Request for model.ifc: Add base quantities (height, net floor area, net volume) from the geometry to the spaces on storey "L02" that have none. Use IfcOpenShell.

First a look at what the model holds.

```python
import ifcopenshell
import ifcopenshell.util.element
import ifcopenshell.util.unit

model = ifcopenshell.open("model.ifc")
print(model.schema)
for unit_type in ("LENGTHUNIT", "AREAUNIT", "VOLUMEUNIT"):
    print(unit_type, ifcopenshell.util.unit.calculate_unit_scale(model, unit_type))
storey = next(s for s in model.by_type("IfcBuildingStorey") if s.Name == "L02")
spaces = [e for e in ifcopenshell.util.element.get_decomposition(storey) if e.is_a("IfcSpace")]
for e in sorted(spaces, key=lambda e: e.id()):
    print(e.id(), e.is_a(), e.Name, list(ifcopenshell.util.element.get_psets(e, qtos_only=True)), sep=" | ")
```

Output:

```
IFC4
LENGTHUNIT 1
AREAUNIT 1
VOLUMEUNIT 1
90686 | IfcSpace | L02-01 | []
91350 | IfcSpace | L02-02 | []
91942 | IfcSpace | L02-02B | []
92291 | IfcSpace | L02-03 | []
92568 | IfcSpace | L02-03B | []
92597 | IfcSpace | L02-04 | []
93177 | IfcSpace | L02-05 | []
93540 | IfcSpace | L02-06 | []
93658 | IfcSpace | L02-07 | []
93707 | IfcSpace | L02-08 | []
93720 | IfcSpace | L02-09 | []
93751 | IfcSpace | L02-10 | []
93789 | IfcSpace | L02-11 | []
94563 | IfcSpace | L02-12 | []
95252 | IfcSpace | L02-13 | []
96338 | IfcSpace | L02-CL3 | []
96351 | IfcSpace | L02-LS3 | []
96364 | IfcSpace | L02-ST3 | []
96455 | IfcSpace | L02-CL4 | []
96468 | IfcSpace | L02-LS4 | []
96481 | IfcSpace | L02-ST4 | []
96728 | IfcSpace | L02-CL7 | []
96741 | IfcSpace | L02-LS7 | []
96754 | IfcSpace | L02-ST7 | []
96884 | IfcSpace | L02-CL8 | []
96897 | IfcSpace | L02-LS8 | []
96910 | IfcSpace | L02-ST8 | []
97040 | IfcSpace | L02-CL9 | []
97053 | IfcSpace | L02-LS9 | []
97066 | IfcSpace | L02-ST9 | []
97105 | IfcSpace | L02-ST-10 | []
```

```python
import ifcopenshell
import ifcopenshell.api.pset
import ifcopenshell.geom
import ifcopenshell.util.element
import ifcopenshell.util.shape
import ifcopenshell.util.unit

model = ifcopenshell.open("model.ifc")
unit_scale = ifcopenshell.util.unit.calculate_unit_scale(model)
area_scale = ifcopenshell.util.unit.calculate_unit_scale(model, "AREAUNIT")
volume_scale = ifcopenshell.util.unit.calculate_unit_scale(model, "VOLUMEUNIT")
settings = ifcopenshell.geom.settings()

storey = next(s for s in model.by_type("IfcBuildingStorey") if s.Name == "L02")
spaces = [e for e in ifcopenshell.util.element.get_decomposition(storey) if e.is_a("IfcSpace")]

for e in sorted(spaces, key=lambda e: e.id()):
    if ifcopenshell.util.element.get_psets(e, qtos_only=True, should_inherit=False):
        continue
    # Geometry comes back in metres, in the element's own axes.
    shape = ifcopenshell.geom.create_shape(settings, e)
    values = {
        "Height": ifcopenshell.util.shape.get_z(shape.geometry) / unit_scale,
        "NetFloorArea": ifcopenshell.util.shape.get_footprint_area(shape.geometry) / area_scale,
        "NetVolume": ifcopenshell.util.shape.get_volume(shape.geometry) / volume_scale,
    }
    qto = ifcopenshell.api.pset.add_qto(model, product=e, name="Qto_SpaceBaseQuantities")
    ifcopenshell.api.pset.edit_qto(model, qto=qto, properties=values)
    print(e.id(), {k: round(v, 3) for k, v in values.items()})

model.write("model_rev.ifc")
```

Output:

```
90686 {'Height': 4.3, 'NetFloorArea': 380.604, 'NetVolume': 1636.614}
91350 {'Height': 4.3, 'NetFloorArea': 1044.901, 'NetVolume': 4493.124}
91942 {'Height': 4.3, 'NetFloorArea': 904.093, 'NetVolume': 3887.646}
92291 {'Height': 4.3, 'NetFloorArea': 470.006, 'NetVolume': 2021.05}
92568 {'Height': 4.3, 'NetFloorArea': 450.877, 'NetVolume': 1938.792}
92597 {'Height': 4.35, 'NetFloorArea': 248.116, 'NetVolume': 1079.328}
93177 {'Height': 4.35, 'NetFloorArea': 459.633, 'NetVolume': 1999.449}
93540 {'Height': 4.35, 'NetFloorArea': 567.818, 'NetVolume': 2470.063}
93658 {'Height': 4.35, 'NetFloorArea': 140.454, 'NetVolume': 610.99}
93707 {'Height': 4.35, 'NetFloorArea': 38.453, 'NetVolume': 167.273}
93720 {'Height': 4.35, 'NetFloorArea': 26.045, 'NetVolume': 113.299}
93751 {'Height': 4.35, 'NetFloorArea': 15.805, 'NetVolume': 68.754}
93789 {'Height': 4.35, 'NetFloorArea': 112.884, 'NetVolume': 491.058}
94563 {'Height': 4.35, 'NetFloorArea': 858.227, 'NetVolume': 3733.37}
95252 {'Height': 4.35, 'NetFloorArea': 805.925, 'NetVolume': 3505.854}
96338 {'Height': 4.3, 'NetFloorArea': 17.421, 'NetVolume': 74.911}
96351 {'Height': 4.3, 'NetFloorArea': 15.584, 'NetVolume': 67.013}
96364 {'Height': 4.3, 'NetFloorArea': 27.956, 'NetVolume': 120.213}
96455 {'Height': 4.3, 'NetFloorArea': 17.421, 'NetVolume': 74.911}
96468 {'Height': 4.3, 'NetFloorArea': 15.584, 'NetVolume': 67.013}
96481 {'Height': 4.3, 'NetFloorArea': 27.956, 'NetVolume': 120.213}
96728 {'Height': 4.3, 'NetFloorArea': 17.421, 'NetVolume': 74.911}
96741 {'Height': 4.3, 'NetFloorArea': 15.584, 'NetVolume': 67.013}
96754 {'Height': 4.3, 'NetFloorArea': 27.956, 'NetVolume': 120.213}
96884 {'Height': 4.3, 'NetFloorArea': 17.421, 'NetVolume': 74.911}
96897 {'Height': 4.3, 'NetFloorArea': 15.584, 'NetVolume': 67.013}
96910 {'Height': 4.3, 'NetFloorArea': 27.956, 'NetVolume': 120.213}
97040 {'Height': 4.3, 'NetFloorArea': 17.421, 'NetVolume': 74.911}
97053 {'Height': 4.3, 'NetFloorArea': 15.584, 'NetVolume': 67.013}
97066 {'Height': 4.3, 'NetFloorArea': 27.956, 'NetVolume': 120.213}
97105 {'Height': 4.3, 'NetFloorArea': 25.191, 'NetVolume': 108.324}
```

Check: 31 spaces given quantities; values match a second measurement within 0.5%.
